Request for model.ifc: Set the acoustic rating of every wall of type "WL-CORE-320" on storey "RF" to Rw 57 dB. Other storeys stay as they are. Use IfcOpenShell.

First a look at what the model holds.

```python
import ifcopenshell
import ifcopenshell.util.element

model = ifcopenshell.open("model.ifc")
print(model.schema)
storey = next(s for s in model.by_type("IfcBuildingStorey") if s.Name == "RF")
walls = [e for e in ifcopenshell.util.element.get_decomposition(storey) if e.is_a("IfcWall")]
seen = {}
for e in walls:
    element_type = ifcopenshell.util.element.get_type(e)
    key = (element_type.Name if element_type != e and element_type else None, ifcopenshell.util.element.get_pset(e, "Pset_WallCommon", "AcousticRating"))
    seen[key] = seen.get(key, 0) + 1
for (name, value), count in sorted(seen.items(), key=str):
    print(count, "x", name, "|", value)
```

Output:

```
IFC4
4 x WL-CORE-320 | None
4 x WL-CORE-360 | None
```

```python
import ifcopenshell
import ifcopenshell.api.pset
import ifcopenshell.util.element

model = ifcopenshell.open("model.ifc")

storey = next(s for s in model.by_type("IfcBuildingStorey") if s.Name == "RF")
walls = [e for e in ifcopenshell.util.element.get_decomposition(storey) if e.is_a("IfcWall")]

count = 0
for e in walls:
    element_type = ifcopenshell.util.element.get_type(e)
    if element_type in (None, e) or element_type.Name != "WL-CORE-320":
        continue
    # add_pset returns the element's existing set when there is one.
    pset = ifcopenshell.api.pset.add_pset(model, product=e, name="Pset_WallCommon")
    ifcopenshell.api.pset.edit_pset(model, pset=pset, properties={"AcousticRating": "Rw 57 dB"})
    count += 1

print(count, "walls updated")

model.write("model_rev.ifc")
```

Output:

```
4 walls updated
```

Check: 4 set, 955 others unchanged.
